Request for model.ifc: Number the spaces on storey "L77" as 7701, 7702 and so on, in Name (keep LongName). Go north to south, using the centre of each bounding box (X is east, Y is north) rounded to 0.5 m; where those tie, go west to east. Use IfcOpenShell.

First a look at what the model holds.

```python
import ifcopenshell
import ifcopenshell.util.element
import ifcopenshell.util.placement

model = ifcopenshell.open("model.ifc")
print(model.schema)
storey = next(s for s in model.by_type("IfcBuildingStorey") if s.Name == "L77")
spaces = [e for e in ifcopenshell.util.element.get_decomposition(storey) if e.is_a("IfcSpace")]
for e in sorted(spaces, key=lambda e: e.id()):
    origin = ifcopenshell.util.placement.get_local_placement(e.ObjectPlacement)[:3, 3]
    print(e.id(), e.Name, e.LongName, origin.round(2) + 0.0, sep=" | ")
```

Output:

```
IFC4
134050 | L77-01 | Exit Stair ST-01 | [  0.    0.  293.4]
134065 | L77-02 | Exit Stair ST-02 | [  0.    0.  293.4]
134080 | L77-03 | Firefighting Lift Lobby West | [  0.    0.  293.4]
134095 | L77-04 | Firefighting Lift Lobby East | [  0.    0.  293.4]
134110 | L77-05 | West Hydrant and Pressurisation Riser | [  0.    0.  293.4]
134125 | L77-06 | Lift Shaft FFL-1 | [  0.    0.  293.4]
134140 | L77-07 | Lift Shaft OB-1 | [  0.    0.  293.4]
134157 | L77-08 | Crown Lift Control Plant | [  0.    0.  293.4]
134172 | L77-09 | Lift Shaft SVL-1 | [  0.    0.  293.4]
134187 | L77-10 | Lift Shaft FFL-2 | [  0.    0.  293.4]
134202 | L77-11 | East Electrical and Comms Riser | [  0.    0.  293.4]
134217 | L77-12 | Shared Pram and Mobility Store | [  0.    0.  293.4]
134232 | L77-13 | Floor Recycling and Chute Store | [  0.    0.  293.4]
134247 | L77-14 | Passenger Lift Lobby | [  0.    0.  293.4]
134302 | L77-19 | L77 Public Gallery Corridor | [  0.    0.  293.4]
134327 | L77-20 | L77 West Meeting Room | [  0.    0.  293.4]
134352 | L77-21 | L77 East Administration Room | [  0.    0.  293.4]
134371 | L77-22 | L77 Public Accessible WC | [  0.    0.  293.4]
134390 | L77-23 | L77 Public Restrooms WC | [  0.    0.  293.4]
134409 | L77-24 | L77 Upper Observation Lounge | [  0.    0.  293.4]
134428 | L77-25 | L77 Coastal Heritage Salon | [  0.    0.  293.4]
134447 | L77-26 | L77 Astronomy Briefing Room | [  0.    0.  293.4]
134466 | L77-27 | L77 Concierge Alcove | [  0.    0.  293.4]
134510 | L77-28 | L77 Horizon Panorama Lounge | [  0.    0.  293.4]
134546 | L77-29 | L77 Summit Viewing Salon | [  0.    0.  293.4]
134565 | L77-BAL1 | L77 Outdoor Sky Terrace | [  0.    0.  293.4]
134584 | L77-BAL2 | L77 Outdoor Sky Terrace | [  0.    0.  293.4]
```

```python
import ifcopenshell
import ifcopenshell.geom
import ifcopenshell.util.element
import ifcopenshell.util.shape

model = ifcopenshell.open("model.ifc")
settings = ifcopenshell.geom.settings()
settings.set("use-world-coords", True)


def centre(element):
    shape = ifcopenshell.geom.create_shape(settings, element)
    return ifcopenshell.util.shape.get_bbox_centroid(shape.geometry)


storey = next(s for s in model.by_type("IfcBuildingStorey") if s.Name == "L77")
spaces = [e for e in ifcopenshell.util.element.get_decomposition(storey) if e.is_a("IfcSpace")]

# Insertion points can sit at a corner or the storey origin, so sort by the geometry (in metres).
centres = {e: centre(e) for e in spaces}
spaces.sort(key=lambda e: (-round(centres[e][1] / 0.5), centres[e][0]))

for i, e in enumerate(spaces, start=1):
    number = f"77{i:02d}"
    e.Name = number
    print(e.id(), number)

model.write("model_edited.ifc")
```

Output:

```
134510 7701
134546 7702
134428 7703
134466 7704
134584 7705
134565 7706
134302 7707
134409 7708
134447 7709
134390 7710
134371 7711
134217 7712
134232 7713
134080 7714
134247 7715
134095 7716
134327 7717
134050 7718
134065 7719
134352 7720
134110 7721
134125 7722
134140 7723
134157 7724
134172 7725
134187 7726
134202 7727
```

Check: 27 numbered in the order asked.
